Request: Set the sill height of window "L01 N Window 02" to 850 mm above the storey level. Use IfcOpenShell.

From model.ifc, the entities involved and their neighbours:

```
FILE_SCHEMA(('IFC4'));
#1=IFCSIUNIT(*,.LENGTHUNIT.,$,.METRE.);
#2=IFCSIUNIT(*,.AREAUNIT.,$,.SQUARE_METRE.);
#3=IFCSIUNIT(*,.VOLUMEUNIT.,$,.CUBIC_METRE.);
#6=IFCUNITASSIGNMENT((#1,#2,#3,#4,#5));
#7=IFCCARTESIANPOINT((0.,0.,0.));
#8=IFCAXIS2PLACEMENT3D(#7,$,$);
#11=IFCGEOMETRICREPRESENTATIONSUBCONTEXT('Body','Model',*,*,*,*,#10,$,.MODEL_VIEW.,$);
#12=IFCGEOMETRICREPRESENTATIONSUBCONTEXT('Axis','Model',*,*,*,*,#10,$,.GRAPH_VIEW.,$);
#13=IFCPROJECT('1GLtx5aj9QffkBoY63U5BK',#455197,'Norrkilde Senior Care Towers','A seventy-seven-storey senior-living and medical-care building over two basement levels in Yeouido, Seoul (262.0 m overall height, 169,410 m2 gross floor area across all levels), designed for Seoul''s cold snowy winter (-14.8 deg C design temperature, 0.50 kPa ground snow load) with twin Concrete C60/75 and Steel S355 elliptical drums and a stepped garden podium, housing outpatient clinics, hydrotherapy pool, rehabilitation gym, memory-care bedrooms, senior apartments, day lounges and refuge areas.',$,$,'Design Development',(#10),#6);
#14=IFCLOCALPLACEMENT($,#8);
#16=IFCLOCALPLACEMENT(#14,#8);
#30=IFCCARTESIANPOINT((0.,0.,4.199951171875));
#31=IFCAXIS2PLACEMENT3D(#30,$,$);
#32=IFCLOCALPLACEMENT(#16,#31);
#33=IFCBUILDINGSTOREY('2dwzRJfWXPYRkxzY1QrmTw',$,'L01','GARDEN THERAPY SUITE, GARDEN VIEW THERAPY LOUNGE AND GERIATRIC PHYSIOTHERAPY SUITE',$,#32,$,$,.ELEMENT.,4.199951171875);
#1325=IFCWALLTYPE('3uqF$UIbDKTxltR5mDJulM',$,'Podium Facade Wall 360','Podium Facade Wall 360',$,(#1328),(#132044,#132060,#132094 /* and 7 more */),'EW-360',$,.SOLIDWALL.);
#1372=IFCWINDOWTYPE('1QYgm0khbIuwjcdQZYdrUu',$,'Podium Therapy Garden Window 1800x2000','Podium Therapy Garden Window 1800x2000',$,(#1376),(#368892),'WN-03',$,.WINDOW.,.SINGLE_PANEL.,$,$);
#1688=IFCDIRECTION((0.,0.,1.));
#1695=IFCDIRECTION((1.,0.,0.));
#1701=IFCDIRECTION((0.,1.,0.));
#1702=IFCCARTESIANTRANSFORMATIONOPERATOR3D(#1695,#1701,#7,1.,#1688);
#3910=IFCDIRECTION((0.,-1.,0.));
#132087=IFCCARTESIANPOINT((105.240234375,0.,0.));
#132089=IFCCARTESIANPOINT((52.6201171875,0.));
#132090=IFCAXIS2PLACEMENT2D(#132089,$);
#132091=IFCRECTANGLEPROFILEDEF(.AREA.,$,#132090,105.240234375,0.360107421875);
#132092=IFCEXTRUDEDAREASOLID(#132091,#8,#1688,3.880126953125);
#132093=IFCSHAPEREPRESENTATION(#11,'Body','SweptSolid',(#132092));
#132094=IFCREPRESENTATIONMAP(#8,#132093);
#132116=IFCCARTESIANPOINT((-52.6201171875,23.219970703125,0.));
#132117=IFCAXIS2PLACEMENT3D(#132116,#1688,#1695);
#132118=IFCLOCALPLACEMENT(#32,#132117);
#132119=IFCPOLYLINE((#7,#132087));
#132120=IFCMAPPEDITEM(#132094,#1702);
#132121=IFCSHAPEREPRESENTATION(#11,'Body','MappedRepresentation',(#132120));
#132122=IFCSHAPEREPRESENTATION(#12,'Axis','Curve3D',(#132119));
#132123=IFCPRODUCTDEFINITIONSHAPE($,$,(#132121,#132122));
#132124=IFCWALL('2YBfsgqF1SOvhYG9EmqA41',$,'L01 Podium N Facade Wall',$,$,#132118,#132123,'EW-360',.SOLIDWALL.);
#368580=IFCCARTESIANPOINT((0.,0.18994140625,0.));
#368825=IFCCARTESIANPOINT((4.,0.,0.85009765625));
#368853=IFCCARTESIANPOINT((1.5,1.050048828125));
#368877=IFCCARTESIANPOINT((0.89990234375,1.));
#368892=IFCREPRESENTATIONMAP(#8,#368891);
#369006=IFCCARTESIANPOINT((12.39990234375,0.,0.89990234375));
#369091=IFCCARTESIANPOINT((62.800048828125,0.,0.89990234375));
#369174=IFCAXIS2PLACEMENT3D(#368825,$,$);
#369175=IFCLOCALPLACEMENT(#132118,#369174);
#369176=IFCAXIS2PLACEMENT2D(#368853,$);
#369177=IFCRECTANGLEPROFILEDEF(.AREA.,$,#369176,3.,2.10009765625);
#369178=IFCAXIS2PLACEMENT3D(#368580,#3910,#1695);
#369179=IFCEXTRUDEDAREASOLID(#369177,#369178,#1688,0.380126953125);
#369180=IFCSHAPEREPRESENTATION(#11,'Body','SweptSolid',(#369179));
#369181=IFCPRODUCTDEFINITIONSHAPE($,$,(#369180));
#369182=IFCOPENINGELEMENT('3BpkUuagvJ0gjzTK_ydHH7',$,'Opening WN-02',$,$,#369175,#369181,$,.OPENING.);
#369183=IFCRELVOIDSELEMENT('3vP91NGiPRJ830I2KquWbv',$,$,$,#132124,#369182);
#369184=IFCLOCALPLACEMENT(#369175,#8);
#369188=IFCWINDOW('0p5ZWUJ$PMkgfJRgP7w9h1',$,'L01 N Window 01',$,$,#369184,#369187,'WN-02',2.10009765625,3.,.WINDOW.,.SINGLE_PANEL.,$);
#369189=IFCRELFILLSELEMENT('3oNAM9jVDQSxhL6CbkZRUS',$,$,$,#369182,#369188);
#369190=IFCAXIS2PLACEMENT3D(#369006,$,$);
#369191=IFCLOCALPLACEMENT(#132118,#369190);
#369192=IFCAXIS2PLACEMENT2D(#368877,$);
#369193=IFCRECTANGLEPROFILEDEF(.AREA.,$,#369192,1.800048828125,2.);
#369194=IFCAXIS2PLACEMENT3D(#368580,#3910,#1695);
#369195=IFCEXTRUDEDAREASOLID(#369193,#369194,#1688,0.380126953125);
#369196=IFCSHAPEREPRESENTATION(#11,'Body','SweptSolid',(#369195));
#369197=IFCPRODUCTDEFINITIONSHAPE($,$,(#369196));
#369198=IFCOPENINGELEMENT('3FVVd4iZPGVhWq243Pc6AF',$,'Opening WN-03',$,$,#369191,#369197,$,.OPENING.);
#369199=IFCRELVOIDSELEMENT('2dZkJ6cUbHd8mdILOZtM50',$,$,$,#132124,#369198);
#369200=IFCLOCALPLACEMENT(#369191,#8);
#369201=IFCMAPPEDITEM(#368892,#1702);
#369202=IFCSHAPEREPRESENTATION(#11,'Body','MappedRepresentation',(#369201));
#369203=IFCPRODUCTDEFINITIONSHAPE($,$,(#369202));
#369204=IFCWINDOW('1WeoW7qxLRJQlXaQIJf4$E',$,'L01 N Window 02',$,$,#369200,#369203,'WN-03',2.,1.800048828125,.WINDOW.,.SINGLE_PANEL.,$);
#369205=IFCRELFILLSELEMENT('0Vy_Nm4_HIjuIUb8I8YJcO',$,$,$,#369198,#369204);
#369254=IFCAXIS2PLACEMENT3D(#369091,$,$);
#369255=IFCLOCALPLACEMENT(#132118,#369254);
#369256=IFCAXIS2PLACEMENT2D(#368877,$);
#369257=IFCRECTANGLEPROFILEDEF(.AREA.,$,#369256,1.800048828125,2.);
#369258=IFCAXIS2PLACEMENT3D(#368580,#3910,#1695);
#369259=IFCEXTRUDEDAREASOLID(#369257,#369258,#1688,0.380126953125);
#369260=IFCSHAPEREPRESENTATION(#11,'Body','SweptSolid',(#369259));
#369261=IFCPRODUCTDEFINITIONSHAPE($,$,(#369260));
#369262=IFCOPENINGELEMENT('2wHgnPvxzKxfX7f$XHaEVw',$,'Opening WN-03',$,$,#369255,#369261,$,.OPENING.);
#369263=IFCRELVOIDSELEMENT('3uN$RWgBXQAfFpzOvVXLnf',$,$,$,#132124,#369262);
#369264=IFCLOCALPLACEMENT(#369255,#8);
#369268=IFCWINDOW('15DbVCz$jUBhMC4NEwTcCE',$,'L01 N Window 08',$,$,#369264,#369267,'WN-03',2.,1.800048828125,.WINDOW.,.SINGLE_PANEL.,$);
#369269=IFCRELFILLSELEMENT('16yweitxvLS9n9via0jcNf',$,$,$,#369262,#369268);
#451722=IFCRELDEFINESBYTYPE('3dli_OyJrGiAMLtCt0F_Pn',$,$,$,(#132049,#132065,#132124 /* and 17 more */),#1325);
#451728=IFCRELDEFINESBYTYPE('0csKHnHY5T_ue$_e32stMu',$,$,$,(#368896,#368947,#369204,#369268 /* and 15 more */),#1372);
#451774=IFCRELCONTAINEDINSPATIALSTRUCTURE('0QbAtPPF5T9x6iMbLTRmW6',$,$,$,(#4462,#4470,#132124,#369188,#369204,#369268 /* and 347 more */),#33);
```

```python
import numpy as np
import ifcopenshell
import ifcopenshell.api.geometry
import ifcopenshell.geom
import ifcopenshell.util.element
import ifcopenshell.util.placement
import ifcopenshell.util.shape
import ifcopenshell.util.unit

model = ifcopenshell.open("model.ifc")
unit_scale = ifcopenshell.util.unit.calculate_unit_scale(model)

window = model.by_guid("1WeoW7qxLRJQlXaQIJf4$E")
opening = window.FillsVoids[0].RelatingOpeningElement
storey = ifcopenshell.util.element.get_container(window, ifc_class="IfcBuildingStorey")
level = ifcopenshell.util.placement.get_local_placement(storey.ObjectPlacement)[2, 3]

# The opening's origin need not be at the sill, so measure its lowest point.
shape = ifcopenshell.geom.create_shape(ifcopenshell.geom.settings(), opening)
bottom = ifcopenshell.util.shape.get_shape_bottom_elevation(shape, shape.geometry) / unit_scale
dz = level + 0.85 / unit_scale - bottom

shift = np.array([0.0, 0.0, dz])
# The window is placed relative to its opening, so it follows when the opening moves.
matrix = ifcopenshell.util.placement.get_local_placement(opening.ObjectPlacement)
matrix[:3, 3] += shift
ifcopenshell.api.geometry.edit_object_placement(
    model, product=opening, matrix=matrix, is_si=False, should_transform_children=True
)

print(f"moved by {dz * unit_scale:+.3f} m")

model.write("model_updated.ifc")
```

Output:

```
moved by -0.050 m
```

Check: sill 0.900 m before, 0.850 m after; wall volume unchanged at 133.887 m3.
